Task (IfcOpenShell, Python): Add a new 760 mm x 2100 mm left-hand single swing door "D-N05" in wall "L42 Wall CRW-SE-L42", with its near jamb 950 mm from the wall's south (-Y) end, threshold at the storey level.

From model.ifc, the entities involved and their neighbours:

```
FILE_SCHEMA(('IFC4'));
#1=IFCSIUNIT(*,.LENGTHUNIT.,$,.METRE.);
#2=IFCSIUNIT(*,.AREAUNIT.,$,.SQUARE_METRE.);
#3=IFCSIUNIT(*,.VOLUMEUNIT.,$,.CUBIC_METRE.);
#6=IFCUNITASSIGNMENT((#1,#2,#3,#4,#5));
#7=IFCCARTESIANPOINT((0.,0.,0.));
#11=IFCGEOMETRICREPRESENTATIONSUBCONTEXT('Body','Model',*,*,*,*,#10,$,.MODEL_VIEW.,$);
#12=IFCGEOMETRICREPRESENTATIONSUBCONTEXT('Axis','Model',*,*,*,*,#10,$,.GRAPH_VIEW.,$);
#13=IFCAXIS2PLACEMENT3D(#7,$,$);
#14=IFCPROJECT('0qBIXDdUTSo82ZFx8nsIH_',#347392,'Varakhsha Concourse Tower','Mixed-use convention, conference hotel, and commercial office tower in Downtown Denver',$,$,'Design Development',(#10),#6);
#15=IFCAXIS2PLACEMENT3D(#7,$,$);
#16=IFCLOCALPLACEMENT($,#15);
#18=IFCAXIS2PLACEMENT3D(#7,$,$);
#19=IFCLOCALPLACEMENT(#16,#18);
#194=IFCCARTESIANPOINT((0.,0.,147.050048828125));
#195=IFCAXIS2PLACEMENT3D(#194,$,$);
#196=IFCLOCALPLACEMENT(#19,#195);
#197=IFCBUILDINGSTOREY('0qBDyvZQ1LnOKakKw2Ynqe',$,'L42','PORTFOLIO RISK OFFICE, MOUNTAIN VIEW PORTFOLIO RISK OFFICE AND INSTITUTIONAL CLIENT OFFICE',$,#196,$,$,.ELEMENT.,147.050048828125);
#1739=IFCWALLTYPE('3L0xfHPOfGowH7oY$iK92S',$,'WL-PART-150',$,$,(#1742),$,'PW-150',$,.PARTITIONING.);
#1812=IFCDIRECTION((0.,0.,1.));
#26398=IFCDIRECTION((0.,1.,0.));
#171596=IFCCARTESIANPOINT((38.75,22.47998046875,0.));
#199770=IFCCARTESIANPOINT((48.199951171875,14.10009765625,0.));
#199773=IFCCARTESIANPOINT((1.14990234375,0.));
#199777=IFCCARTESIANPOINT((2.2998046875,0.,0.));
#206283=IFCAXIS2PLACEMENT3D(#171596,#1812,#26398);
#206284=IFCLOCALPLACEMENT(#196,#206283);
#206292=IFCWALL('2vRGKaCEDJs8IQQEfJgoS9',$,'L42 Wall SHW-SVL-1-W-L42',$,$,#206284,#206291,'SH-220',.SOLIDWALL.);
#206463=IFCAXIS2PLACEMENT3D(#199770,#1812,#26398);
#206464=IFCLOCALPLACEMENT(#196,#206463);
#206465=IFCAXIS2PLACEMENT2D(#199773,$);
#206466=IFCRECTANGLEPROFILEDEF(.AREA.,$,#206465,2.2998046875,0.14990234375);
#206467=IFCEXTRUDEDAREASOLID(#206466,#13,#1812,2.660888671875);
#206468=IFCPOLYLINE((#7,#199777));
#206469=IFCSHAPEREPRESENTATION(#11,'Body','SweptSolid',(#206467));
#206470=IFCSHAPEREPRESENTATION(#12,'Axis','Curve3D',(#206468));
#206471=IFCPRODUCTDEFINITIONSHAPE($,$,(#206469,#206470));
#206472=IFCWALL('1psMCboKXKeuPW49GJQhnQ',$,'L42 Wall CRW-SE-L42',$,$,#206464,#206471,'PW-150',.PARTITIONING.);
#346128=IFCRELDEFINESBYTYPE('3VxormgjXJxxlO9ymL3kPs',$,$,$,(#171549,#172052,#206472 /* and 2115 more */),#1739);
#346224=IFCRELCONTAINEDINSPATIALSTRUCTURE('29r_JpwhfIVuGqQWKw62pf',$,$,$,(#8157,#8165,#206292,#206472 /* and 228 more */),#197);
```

```python
import numpy as np
import ifcopenshell
import ifcopenshell.api.feature
import ifcopenshell.api.geometry
import ifcopenshell.api.root
import ifcopenshell.api.spatial
import ifcopenshell.geom
import ifcopenshell.util.element
import ifcopenshell.util.placement
import ifcopenshell.util.representation
import ifcopenshell.util.shape
import ifcopenshell.util.unit

model = ifcopenshell.open("model.ifc")
unit_scale = ifcopenshell.util.unit.calculate_unit_scale(model)
settings = ifcopenshell.geom.settings()


def volume(element):
    """Net volume in cubic metres, openings subtracted."""
    shape = ifcopenshell.geom.create_shape(settings, element)
    return ifcopenshell.util.shape.get_volume(shape.geometry)


wall = model.by_guid("1psMCboKXKeuPW49GJQhnQ")
storey = ifcopenshell.util.element.get_container(wall, ifc_class="IfcBuildingStorey")
context = ifcopenshell.util.representation.get_context(model, "Model", "Body", "MODEL_VIEW")
before = volume(wall)

width, height, from_end, sill = 0.76, 2.1, 0.95, 0.0  # metres

# The wall runs along its own X axis, and the end named is its -X end.
wall_shape = ifcopenshell.geom.create_shape(settings, wall)
x, y, z = ifcopenshell.util.shape.get_vertices(wall_shape.geometry).T
start = x.min() + from_end
face, thickness = float(y.min()), float(y.max() - y.min())
wall_matrix = ifcopenshell.util.placement.get_local_placement(wall.ObjectPlacement)
level = ifcopenshell.util.placement.get_local_placement(storey.ObjectPlacement)[2, 3]


def in_wall(x, y):
    """Placement at x, y metres in the wall's axes, at sill height."""
    matrix = wall_matrix.copy()
    matrix[:, 3] = wall_matrix @ np.array([x / unit_scale, y / unit_scale, 0.0, 1.0])
    matrix[2, 3] = level + sill / unit_scale
    return matrix


# Opening: a box that overshoots both wall faces by 50 mm.
opening = ifcopenshell.api.root.create_entity(model, ifc_class="IfcOpeningElement", predefined_type="OPENING")
box = ifcopenshell.api.geometry.add_wall_representation(
    model, context=context, length=width, height=height, thickness=thickness + 0.1
)
ifcopenshell.api.geometry.assign_representation(model, product=opening, representation=box)
ifcopenshell.api.geometry.edit_object_placement(model, product=opening, matrix=in_wall(start, face - 0.05), is_si=False)
ifcopenshell.api.feature.add_feature(model, feature=opening, element=wall)

door = ifcopenshell.api.root.create_entity(model, ifc_class="IfcDoor", name="D-N05", predefined_type="DOOR")
door.OverallWidth, door.OverallHeight = width / unit_scale, height / unit_scale
door.OperationType = "SINGLE_SWING_LEFT"
body = ifcopenshell.api.geometry.add_door_representation(
    model,
    context=context,
    overall_width=door.OverallWidth,
    overall_height=door.OverallHeight,
    operation_type="SINGLE_SWING_LEFT",
    lining_properties={"LiningDepth": thickness / unit_scale, "ThresholdDepth": thickness / unit_scale},
)
ifcopenshell.api.geometry.assign_representation(model, product=door, representation=body)
ifcopenshell.api.spatial.assign_container(model, products=[door], relating_structure=storey)
ifcopenshell.api.feature.add_filling(model, opening=opening, element=door)

# The lining spans the wall, so the door starts at the wall face.
ifcopenshell.api.geometry.edit_object_placement(model, product=door, matrix=in_wall(start, face), is_si=False)

after = volume(wall)

print(f"wall volume {before:.3f} -> {after:.3f} m3")

model.write("model_edited.ifc")
```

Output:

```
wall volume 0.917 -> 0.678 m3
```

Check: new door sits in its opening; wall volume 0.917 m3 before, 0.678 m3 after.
